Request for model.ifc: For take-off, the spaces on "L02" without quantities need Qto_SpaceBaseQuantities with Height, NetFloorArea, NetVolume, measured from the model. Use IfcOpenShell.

First a look at what the model holds.

```python
import ifcopenshell
import ifcopenshell.util.element
import ifcopenshell.util.unit

model = ifcopenshell.open("model.ifc")
print(model.schema)
for unit_type in ("LENGTHUNIT", "AREAUNIT", "VOLUMEUNIT"):
    print(unit_type, ifcopenshell.util.unit.calculate_unit_scale(model, unit_type))
storey = next(s for s in model.by_type("IfcBuildingStorey") if s.Name == "L02")
spaces = [e for e in ifcopenshell.util.element.get_decomposition(storey) if e.is_a("IfcSpace")]
for e in sorted(spaces, key=lambda e: e.id()):
    print(e.id(), e.is_a(), e.Name, list(ifcopenshell.util.element.get_psets(e, qtos_only=True)), sep=" | ")
```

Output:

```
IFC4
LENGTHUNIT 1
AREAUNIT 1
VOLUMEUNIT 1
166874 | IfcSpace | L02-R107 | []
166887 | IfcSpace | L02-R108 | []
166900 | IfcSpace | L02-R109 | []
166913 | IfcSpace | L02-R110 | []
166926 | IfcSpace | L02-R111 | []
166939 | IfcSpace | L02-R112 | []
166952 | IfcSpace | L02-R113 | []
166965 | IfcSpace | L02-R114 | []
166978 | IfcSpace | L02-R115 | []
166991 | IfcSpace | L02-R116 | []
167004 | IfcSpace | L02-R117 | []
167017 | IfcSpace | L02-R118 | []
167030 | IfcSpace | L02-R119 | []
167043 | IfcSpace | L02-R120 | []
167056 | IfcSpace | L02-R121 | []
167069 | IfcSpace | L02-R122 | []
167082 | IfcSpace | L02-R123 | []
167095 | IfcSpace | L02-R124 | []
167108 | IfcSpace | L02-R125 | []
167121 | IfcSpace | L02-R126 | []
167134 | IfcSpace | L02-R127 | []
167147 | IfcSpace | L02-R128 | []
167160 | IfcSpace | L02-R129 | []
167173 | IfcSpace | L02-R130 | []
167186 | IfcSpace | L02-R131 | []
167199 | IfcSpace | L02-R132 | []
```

```python
import ifcopenshell
import ifcopenshell.api.pset
import ifcopenshell.geom
import ifcopenshell.util.element
import ifcopenshell.util.shape
import ifcopenshell.util.unit

model = ifcopenshell.open("model.ifc")
unit_scale = ifcopenshell.util.unit.calculate_unit_scale(model)
area_scale = ifcopenshell.util.unit.calculate_unit_scale(model, "AREAUNIT")
volume_scale = ifcopenshell.util.unit.calculate_unit_scale(model, "VOLUMEUNIT")
settings = ifcopenshell.geom.settings()

storey = next(s for s in model.by_type("IfcBuildingStorey") if s.Name == "L02")
spaces = [e for e in ifcopenshell.util.element.get_decomposition(storey) if e.is_a("IfcSpace")]

for e in sorted(spaces, key=lambda e: e.id()):
    if ifcopenshell.util.element.get_psets(e, qtos_only=True, should_inherit=False):
        continue
    # Geometry comes back in metres, in the element's own axes.
    shape = ifcopenshell.geom.create_shape(settings, e)
    values = {
        "Height": ifcopenshell.util.shape.get_z(shape.geometry) / unit_scale,
        "NetFloorArea": ifcopenshell.util.shape.get_footprint_area(shape.geometry) / area_scale,
        "NetVolume": ifcopenshell.util.shape.get_volume(shape.geometry) / volume_scale,
    }
    qto = ifcopenshell.api.pset.add_qto(model, product=e, name="Qto_SpaceBaseQuantities")
    ifcopenshell.api.pset.edit_qto(model, qto=qto, properties=values)
    print(e.id(), {k: round(v, 3) for k, v in values.items()})

model.write("model_v2.ifc")
```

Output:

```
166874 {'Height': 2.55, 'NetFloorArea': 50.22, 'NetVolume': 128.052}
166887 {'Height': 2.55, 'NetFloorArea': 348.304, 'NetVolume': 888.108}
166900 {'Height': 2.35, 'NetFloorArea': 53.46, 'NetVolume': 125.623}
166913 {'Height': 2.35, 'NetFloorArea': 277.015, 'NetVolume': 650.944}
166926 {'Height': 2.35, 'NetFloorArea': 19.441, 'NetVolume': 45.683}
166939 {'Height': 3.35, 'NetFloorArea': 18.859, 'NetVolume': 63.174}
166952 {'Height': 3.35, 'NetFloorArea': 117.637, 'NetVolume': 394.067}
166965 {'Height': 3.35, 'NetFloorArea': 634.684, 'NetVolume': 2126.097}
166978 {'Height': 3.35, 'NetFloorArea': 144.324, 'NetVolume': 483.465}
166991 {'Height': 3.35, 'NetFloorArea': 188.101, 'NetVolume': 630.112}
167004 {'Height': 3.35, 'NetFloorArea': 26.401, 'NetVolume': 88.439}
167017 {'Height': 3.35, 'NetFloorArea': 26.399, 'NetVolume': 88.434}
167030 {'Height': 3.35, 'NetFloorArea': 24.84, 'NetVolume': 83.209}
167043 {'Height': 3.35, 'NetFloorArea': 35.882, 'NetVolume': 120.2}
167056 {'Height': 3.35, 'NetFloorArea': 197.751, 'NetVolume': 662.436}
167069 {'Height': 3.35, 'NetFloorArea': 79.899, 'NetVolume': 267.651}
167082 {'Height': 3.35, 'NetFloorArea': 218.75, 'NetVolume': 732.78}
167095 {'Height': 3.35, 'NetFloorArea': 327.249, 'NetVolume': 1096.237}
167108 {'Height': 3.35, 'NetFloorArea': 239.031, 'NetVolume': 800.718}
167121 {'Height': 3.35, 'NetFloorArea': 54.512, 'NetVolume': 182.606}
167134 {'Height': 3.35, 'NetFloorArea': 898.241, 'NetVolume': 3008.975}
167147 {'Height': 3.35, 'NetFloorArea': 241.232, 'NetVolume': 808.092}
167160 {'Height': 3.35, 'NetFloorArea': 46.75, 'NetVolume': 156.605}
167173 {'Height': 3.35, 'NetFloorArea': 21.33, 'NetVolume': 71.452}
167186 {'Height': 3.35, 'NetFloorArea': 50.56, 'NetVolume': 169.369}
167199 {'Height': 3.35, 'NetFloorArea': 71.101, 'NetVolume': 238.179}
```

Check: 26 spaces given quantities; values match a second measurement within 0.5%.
